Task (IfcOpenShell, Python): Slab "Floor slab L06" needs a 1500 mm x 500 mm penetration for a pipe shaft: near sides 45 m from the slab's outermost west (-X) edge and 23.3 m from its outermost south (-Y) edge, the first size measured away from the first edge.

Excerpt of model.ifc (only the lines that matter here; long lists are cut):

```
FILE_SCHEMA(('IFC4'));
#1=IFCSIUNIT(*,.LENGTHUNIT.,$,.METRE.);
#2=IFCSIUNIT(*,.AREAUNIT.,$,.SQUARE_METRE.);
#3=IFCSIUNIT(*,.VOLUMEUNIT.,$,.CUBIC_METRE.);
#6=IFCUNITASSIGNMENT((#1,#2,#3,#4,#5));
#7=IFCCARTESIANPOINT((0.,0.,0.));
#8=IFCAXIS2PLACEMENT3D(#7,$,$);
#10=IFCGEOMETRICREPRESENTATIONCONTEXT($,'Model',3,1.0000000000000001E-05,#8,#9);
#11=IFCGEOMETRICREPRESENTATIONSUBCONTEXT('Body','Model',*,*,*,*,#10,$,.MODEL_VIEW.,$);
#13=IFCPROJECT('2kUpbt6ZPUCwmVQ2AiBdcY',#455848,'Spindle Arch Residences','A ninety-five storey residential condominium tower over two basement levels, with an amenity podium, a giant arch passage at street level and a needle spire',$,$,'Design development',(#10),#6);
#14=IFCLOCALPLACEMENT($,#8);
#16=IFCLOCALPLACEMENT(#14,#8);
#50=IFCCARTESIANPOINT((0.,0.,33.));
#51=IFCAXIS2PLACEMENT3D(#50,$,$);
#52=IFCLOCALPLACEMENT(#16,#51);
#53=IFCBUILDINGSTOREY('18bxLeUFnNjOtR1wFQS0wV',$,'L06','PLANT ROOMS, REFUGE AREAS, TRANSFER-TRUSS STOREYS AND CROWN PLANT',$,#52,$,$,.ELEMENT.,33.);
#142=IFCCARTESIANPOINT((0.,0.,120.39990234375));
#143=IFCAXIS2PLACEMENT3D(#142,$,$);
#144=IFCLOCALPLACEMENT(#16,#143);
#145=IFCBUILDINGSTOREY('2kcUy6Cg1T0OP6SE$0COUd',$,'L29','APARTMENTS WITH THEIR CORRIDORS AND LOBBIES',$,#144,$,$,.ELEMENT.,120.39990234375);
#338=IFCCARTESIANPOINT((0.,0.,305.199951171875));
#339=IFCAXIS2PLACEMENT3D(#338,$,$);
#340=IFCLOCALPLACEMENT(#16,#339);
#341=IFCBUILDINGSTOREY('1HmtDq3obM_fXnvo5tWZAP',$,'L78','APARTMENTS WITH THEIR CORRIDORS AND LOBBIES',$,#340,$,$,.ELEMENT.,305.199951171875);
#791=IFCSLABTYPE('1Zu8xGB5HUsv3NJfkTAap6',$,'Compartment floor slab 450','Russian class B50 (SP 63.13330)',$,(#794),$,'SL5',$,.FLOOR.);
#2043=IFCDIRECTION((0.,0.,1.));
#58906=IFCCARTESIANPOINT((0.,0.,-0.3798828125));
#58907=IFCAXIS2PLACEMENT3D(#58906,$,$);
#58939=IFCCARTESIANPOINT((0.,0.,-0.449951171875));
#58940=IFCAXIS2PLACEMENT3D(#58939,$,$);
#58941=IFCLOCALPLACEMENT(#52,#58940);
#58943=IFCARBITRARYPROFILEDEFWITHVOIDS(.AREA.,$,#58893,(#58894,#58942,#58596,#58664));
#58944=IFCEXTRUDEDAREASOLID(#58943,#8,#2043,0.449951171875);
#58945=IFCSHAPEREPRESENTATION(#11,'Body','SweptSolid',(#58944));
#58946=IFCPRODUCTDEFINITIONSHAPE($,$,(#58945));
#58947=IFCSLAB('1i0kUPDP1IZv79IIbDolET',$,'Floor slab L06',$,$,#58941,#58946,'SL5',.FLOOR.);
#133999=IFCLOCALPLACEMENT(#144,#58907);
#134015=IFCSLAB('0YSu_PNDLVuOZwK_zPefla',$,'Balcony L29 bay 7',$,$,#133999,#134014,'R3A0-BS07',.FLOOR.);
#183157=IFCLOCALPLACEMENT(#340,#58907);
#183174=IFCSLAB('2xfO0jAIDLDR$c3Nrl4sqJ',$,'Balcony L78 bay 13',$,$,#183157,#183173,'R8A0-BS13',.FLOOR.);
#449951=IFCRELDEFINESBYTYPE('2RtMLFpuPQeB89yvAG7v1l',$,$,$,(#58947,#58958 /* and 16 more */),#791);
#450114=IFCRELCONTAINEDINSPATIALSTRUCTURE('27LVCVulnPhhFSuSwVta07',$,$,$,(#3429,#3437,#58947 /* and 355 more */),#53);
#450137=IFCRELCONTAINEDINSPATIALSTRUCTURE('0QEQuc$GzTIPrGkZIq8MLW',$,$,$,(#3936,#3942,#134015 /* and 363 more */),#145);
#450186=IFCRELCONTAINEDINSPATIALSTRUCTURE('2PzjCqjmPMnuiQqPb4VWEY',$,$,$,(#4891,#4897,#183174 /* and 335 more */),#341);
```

```python
import numpy as np
import ifcopenshell
import ifcopenshell.api.feature
import ifcopenshell.api.geometry
import ifcopenshell.api.root
import ifcopenshell.geom
import ifcopenshell.util.placement
import ifcopenshell.util.representation
import ifcopenshell.util.shape
import ifcopenshell.util.unit

model = ifcopenshell.open("model.ifc")
unit_scale = ifcopenshell.util.unit.calculate_unit_scale(model)
settings = ifcopenshell.geom.settings()


def volume(element):
    """Net volume in cubic metres, openings subtracted."""
    shape = ifcopenshell.geom.create_shape(settings, element)
    return ifcopenshell.util.shape.get_volume(shape.geometry)


slab = model.by_guid("1i0kUPDP1IZv79IIbDolET")
before = volume(slab)

# Extent in the slab's own axes, in metres. The edges named are its -X and -Y sides.
slab_shape = ifcopenshell.geom.create_shape(settings, slab)
vertices = ifcopenshell.util.shape.get_vertices(slab_shape.geometry)
x_min, y_min, bottom = vertices.min(axis=0)
top = vertices[:, 2].max()

opening = ifcopenshell.api.root.create_entity(model, ifc_class="IfcOpeningElement", name="Pipe shaft opening", predefined_type="OPENING")
context = ifcopenshell.util.representation.get_context(model, "Model", "Body", "MODEL_VIEW")
width, depth = 1.5, 0.5
outline = [(0.0, 0.0), (width, 0.0), (width, depth), (0.0, depth), (0.0, 0.0)]
# Overshoot both faces by 50 mm so the cut is clean.
shape = ifcopenshell.api.geometry.add_slab_representation(
    model, context=context, depth=top - bottom + 0.1, polyline=outline
)
ifcopenshell.api.geometry.assign_representation(model, product=opening, representation=shape)

matrix = ifcopenshell.util.placement.get_local_placement(slab.ObjectPlacement)
matrix[:, 3] = matrix @ np.append(np.array([x_min + 45, y_min + 23.3, bottom - 0.05]) / unit_scale, 1.0)
ifcopenshell.api.geometry.edit_object_placement(model, product=opening, matrix=matrix, is_si=False)
ifcopenshell.api.feature.add_feature(model, feature=opening, element=slab)

after = volume(slab)

print(f"slab volume {before:.3f} -> {after:.3f} m3")

model.write("model_rev.ifc")
```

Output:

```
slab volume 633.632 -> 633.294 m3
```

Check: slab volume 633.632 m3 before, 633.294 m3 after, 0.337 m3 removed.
